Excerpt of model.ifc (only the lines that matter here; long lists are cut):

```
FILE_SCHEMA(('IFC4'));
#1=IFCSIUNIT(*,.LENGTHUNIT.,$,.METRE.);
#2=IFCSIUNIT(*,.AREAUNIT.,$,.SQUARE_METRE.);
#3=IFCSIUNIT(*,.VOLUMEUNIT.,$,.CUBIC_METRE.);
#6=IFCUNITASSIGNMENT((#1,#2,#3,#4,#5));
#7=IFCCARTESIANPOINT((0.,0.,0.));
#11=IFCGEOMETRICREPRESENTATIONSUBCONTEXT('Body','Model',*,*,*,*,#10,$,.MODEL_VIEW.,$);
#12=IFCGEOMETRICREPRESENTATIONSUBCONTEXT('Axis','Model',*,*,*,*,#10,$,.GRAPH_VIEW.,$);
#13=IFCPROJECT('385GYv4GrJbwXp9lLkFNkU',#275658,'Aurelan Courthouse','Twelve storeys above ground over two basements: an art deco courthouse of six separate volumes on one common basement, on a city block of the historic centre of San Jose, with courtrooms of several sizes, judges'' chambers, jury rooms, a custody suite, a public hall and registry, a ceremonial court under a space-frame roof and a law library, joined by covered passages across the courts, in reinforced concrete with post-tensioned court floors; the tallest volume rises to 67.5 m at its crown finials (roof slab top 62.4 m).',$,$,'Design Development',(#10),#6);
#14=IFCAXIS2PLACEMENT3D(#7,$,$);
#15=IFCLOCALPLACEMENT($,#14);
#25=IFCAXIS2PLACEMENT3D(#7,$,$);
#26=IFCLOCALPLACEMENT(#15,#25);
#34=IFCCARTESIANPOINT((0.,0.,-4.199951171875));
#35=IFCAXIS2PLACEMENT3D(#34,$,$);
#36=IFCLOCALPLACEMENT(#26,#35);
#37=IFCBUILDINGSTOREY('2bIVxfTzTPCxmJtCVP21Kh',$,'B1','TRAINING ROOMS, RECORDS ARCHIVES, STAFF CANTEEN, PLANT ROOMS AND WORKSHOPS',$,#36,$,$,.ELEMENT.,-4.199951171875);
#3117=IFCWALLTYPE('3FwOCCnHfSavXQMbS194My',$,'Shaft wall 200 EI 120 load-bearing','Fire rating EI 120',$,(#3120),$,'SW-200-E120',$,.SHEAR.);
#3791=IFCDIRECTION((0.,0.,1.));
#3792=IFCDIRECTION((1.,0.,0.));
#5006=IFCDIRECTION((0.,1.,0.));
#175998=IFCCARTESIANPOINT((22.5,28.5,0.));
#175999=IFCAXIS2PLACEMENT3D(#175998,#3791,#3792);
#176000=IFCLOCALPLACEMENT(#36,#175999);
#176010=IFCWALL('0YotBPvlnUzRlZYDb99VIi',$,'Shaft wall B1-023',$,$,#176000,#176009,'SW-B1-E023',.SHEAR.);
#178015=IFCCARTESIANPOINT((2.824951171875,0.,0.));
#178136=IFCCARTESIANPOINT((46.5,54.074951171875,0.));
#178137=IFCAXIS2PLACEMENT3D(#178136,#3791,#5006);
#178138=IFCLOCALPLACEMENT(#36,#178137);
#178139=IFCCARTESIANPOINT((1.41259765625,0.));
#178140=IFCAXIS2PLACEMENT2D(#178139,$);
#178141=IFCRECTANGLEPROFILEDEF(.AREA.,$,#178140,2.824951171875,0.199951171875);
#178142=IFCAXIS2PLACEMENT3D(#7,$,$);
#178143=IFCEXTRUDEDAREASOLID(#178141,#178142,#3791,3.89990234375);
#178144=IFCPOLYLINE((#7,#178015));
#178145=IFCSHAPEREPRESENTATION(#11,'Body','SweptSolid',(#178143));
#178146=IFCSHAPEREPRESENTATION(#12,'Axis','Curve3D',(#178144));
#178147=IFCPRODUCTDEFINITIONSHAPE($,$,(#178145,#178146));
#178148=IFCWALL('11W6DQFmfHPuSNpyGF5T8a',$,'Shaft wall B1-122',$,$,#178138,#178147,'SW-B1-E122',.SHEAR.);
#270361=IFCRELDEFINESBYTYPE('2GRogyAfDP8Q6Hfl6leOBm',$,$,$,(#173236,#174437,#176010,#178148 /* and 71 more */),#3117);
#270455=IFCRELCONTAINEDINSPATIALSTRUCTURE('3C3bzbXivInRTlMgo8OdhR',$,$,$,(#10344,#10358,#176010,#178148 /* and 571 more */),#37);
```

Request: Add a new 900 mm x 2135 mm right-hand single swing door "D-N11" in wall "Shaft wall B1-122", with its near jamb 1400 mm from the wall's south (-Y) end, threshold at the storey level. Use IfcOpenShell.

```python
import numpy as np
import ifcopenshell
import ifcopenshell.api.feature
import ifcopenshell.api.geometry
import ifcopenshell.api.root
import ifcopenshell.api.spatial
import ifcopenshell.geom
import ifcopenshell.util.element
import ifcopenshell.util.placement
import ifcopenshell.util.representation
import ifcopenshell.util.shape
import ifcopenshell.util.unit

model = ifcopenshell.open("model.ifc")
unit_scale = ifcopenshell.util.unit.calculate_unit_scale(model)
settings = ifcopenshell.geom.settings()


def volume(element):
    """Net volume in cubic metres, openings subtracted."""
    shape = ifcopenshell.geom.create_shape(settings, element)
    return ifcopenshell.util.shape.get_volume(shape.geometry)


wall = model.by_guid("11W6DQFmfHPuSNpyGF5T8a")
storey = ifcopenshell.util.element.get_container(wall, ifc_class="IfcBuildingStorey")
context = ifcopenshell.util.representation.get_context(model, "Model", "Body", "MODEL_VIEW")
before = volume(wall)

width, height, from_end, sill = 0.9, 2.135, 1.4, 0.0  # metres

# The wall runs along its own X axis, and the end named is its -X end.
wall_shape = ifcopenshell.geom.create_shape(settings, wall)
x, y, z = ifcopenshell.util.shape.get_vertices(wall_shape.geometry).T
start = x.min() + from_end
face, thickness = float(y.min()), float(y.max() - y.min())
wall_matrix = ifcopenshell.util.placement.get_local_placement(wall.ObjectPlacement)
level = ifcopenshell.util.placement.get_local_placement(storey.ObjectPlacement)[2, 3]


def in_wall(x, y):
    """Placement at x, y metres in the wall's axes, at sill height."""
    matrix = wall_matrix.copy()
    matrix[:, 3] = wall_matrix @ np.array([x / unit_scale, y / unit_scale, 0.0, 1.0])
    matrix[2, 3] = level + sill / unit_scale
    return matrix


# Opening: a box that overshoots both wall faces by 50 mm.
opening = ifcopenshell.api.root.create_entity(model, ifc_class="IfcOpeningElement", predefined_type="OPENING")
box = ifcopenshell.api.geometry.add_wall_representation(
    model, context=context, length=width, height=height, thickness=thickness + 0.1
)
ifcopenshell.api.geometry.assign_representation(model, product=opening, representation=box)
ifcopenshell.api.geometry.edit_object_placement(model, product=opening, matrix=in_wall(start, face - 0.05), is_si=False)
ifcopenshell.api.feature.add_feature(model, feature=opening, element=wall)

door = ifcopenshell.api.root.create_entity(model, ifc_class="IfcDoor", name="D-N11", predefined_type="DOOR")
door.OverallWidth, door.OverallHeight = width / unit_scale, height / unit_scale
door.OperationType = "SINGLE_SWING_RIGHT"
body = ifcopenshell.api.geometry.add_door_representation(
    model,
    context=context,
    overall_width=door.OverallWidth,
    overall_height=door.OverallHeight,
    operation_type="SINGLE_SWING_RIGHT",
    lining_properties={"LiningDepth": thickness / unit_scale, "ThresholdDepth": thickness / unit_scale},
)
ifcopenshell.api.geometry.assign_representation(model, product=door, representation=body)
ifcopenshell.api.spatial.assign_container(model, products=[door], relating_structure=storey)
ifcopenshell.api.feature.add_filling(model, opening=opening, element=door)

# The lining spans the wall, so the door starts at the wall face.
ifcopenshell.api.geometry.edit_object_placement(model, product=door, matrix=in_wall(start, face), is_si=False)

after = volume(wall)

print(f"wall volume {before:.3f} -> {after:.3f} m3")

model.write("model_v2.ifc")
```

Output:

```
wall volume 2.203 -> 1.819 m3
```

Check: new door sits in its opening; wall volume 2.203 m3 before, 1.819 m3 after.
